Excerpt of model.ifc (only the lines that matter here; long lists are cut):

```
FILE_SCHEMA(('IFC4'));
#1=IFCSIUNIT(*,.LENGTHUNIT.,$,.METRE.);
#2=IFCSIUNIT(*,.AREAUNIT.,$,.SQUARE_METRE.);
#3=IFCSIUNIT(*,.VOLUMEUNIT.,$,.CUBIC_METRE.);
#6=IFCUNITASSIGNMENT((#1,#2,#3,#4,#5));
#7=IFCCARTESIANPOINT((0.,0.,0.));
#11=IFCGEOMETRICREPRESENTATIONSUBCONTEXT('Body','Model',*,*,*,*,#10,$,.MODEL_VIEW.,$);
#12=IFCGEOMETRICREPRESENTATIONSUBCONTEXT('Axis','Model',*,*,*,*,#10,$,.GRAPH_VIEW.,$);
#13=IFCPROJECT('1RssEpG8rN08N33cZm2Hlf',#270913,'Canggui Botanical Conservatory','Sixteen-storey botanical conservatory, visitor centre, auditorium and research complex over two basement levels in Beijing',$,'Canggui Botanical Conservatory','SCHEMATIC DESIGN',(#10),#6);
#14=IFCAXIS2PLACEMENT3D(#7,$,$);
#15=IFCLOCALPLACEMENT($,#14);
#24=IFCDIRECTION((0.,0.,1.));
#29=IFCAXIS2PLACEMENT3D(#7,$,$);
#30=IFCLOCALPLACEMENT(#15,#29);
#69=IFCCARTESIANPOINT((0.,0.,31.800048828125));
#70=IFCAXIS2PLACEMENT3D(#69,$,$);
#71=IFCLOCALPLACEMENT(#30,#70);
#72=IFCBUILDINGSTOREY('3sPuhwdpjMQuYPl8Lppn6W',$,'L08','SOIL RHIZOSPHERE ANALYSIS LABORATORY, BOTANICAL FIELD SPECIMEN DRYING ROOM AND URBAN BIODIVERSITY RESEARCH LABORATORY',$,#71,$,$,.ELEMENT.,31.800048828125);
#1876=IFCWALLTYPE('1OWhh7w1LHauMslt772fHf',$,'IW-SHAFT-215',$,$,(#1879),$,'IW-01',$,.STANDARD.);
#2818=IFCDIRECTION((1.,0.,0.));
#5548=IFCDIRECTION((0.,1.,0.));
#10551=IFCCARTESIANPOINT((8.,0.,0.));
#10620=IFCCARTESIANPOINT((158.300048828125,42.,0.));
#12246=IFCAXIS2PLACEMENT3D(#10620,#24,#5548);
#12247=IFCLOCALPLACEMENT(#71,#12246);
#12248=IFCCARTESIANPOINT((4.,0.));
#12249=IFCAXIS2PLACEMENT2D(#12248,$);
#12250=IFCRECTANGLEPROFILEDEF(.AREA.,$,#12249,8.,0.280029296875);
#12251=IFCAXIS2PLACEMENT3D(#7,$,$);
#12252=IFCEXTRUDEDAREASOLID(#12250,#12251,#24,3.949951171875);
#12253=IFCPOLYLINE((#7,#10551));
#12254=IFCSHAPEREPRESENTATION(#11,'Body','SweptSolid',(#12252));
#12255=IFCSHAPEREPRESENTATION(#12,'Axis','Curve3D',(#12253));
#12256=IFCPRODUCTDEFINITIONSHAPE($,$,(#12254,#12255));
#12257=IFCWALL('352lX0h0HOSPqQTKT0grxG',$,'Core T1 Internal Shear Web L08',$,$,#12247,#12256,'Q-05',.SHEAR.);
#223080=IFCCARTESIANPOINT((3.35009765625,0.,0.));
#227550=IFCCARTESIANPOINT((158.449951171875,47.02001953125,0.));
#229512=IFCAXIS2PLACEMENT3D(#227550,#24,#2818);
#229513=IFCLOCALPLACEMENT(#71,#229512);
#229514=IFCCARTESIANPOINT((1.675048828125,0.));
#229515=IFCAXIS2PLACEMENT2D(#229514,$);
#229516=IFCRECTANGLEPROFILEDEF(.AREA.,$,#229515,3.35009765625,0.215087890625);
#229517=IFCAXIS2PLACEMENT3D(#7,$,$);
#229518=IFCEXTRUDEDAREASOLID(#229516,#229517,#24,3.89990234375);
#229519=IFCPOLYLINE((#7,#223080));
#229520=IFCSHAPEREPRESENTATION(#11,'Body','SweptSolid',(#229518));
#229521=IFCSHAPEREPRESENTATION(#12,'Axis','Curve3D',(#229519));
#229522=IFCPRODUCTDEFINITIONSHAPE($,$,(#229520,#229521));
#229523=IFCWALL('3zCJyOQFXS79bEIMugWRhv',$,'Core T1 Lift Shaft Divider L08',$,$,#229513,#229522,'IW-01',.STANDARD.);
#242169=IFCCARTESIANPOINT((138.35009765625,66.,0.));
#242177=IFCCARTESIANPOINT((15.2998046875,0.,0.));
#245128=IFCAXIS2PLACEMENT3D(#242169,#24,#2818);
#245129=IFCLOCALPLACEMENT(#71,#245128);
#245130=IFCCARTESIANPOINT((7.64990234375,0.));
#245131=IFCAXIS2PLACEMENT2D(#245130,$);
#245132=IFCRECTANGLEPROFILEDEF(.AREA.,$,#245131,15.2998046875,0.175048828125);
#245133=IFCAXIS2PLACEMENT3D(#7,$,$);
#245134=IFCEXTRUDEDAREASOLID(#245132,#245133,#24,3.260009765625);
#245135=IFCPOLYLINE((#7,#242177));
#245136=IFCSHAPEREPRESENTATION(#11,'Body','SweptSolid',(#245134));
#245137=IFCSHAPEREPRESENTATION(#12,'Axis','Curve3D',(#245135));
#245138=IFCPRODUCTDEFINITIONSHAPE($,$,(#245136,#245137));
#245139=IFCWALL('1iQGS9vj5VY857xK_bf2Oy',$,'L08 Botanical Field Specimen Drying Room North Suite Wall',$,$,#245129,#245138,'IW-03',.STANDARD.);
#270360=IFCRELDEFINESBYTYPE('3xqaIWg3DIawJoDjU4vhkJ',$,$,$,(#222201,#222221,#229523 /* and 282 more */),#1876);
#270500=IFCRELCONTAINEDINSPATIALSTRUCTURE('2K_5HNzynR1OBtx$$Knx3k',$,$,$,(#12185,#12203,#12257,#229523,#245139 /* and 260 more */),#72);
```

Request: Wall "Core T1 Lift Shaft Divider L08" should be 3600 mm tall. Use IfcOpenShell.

```python
import ifcopenshell
import ifcopenshell.geom
import ifcopenshell.util.representation
import ifcopenshell.util.shape

model = ifcopenshell.open("model.ifc")
settings = ifcopenshell.geom.settings()


def volume(element):
    """Net volume in cubic metres, openings subtracted."""
    shape = ifcopenshell.geom.create_shape(settings, element)
    return ifcopenshell.util.shape.get_volume(shape.geometry)


wall = model.by_guid("3zCJyOQFXS79bEIMugWRhv")
before = volume(wall)

body = ifcopenshell.util.representation.get_representation(wall, "Model", "Body")
solid = body.Items[0]
old_height = solid.Depth
solid.Depth = 3.6
after = volume(wall)

print(f"height {old_height:g} -> {solid.Depth:g}, volume {before:.3f} -> {after:.3f} m3")

model.write("model_v2.ifc")
```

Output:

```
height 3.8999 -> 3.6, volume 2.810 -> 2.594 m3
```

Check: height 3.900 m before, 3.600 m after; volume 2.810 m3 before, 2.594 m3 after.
